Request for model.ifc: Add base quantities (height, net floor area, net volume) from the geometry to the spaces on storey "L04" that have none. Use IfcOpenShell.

First a look at what the model holds.

```python
import ifcopenshell
import ifcopenshell.util.element
import ifcopenshell.util.unit

model = ifcopenshell.open("model.ifc")
print(model.schema)
for unit_type in ("LENGTHUNIT", "AREAUNIT", "VOLUMEUNIT"):
    print(unit_type, ifcopenshell.util.unit.calculate_unit_scale(model, unit_type))
storey = next(s for s in model.by_type("IfcBuildingStorey") if s.Name == "L04")
spaces = [e for e in ifcopenshell.util.element.get_decomposition(storey) if e.is_a("IfcSpace")]
for e in sorted(spaces, key=lambda e: e.id()):
    print(e.id(), e.is_a(), e.Name, list(ifcopenshell.util.element.get_psets(e, qtos_only=True)), sep=" | ")
```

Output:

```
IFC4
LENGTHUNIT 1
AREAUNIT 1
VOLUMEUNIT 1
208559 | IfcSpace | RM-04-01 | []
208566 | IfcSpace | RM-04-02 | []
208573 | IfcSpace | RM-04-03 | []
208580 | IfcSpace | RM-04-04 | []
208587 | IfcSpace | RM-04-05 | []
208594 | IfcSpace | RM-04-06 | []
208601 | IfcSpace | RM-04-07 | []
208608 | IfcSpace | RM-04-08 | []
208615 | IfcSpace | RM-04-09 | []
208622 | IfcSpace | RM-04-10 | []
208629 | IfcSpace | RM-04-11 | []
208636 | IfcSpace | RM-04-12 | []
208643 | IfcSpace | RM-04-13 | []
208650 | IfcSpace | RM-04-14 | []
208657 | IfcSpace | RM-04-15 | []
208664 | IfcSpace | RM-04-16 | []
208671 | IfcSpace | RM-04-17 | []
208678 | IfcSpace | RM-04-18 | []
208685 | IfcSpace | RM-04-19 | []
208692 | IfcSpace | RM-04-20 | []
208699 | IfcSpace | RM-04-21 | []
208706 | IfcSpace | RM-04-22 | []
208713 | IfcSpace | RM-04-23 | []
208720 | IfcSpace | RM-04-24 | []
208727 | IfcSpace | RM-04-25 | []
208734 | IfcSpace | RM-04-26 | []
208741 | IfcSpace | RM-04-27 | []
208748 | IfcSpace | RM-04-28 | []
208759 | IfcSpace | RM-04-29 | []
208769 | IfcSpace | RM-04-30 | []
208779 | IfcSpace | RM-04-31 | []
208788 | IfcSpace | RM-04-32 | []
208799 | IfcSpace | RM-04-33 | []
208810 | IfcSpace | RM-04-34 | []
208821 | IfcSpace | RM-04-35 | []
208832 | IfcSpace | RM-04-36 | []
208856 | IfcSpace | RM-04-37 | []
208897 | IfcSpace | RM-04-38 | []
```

```python
import ifcopenshell
import ifcopenshell.api.pset
import ifcopenshell.geom
import ifcopenshell.util.element
import ifcopenshell.util.shape
import ifcopenshell.util.unit

model = ifcopenshell.open("model.ifc")
unit_scale = ifcopenshell.util.unit.calculate_unit_scale(model)
area_scale = ifcopenshell.util.unit.calculate_unit_scale(model, "AREAUNIT")
volume_scale = ifcopenshell.util.unit.calculate_unit_scale(model, "VOLUMEUNIT")
settings = ifcopenshell.geom.settings()

storey = next(s for s in model.by_type("IfcBuildingStorey") if s.Name == "L04")
spaces = [e for e in ifcopenshell.util.element.get_decomposition(storey) if e.is_a("IfcSpace")]

for e in sorted(spaces, key=lambda e: e.id()):
    if ifcopenshell.util.element.get_psets(e, qtos_only=True, should_inherit=False):
        continue
    # Geometry comes back in metres, in the element's own axes.
    shape = ifcopenshell.geom.create_shape(settings, e)
    values = {
        "Height": ifcopenshell.util.shape.get_z(shape.geometry) / unit_scale,
        "NetFloorArea": ifcopenshell.util.shape.get_footprint_area(shape.geometry) / area_scale,
        "NetVolume": ifcopenshell.util.shape.get_volume(shape.geometry) / volume_scale,
    }
    qto = ifcopenshell.api.pset.add_qto(model, product=e, name="Qto_SpaceBaseQuantities")
    ifcopenshell.api.pset.edit_qto(model, qto=qto, properties=values)
    print(e.id(), {k: round(v, 3) for k, v in values.items()})

model.write("model_v2.ifc")
```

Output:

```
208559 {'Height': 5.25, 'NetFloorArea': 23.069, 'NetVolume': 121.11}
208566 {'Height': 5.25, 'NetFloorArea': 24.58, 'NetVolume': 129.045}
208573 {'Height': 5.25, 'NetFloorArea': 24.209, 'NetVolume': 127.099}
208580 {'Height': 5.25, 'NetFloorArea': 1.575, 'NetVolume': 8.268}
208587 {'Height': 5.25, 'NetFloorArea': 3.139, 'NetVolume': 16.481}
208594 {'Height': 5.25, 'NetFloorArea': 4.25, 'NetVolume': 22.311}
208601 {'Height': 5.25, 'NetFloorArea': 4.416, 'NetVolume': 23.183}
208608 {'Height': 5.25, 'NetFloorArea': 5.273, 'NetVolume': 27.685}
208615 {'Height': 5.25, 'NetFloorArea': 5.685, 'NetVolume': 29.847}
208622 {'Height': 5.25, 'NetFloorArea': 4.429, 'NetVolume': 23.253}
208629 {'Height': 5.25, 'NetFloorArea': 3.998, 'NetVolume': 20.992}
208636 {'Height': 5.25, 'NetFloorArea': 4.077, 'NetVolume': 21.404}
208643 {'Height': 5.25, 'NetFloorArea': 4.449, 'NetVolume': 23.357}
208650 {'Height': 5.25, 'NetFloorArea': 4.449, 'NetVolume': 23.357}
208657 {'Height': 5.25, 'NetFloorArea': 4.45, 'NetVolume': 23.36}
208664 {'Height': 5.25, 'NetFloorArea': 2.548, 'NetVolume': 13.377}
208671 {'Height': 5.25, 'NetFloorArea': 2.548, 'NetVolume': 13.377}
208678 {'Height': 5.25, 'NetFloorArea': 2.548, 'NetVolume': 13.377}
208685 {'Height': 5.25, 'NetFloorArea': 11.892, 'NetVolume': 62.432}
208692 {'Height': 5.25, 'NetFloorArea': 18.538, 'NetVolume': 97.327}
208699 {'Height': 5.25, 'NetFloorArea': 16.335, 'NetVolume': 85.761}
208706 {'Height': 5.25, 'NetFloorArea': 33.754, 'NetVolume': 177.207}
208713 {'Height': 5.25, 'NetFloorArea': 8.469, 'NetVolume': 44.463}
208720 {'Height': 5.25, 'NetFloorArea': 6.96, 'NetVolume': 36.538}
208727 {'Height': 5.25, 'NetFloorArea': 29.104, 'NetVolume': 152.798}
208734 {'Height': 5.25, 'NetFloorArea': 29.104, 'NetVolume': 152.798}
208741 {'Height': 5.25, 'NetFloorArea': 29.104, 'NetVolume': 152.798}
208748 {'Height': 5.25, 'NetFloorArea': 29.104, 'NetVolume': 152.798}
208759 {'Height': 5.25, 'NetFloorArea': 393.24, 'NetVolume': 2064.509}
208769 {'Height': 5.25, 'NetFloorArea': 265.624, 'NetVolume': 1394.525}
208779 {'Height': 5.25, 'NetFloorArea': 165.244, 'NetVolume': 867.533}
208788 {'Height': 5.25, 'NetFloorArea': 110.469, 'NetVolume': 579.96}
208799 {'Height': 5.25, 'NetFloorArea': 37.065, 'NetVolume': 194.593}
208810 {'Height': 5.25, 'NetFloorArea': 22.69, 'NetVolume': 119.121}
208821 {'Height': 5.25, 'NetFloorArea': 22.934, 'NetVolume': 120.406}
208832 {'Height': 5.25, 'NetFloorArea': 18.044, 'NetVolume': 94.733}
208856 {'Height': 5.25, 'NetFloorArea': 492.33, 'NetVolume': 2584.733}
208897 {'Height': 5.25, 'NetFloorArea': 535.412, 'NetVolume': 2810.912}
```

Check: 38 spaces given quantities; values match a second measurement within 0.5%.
